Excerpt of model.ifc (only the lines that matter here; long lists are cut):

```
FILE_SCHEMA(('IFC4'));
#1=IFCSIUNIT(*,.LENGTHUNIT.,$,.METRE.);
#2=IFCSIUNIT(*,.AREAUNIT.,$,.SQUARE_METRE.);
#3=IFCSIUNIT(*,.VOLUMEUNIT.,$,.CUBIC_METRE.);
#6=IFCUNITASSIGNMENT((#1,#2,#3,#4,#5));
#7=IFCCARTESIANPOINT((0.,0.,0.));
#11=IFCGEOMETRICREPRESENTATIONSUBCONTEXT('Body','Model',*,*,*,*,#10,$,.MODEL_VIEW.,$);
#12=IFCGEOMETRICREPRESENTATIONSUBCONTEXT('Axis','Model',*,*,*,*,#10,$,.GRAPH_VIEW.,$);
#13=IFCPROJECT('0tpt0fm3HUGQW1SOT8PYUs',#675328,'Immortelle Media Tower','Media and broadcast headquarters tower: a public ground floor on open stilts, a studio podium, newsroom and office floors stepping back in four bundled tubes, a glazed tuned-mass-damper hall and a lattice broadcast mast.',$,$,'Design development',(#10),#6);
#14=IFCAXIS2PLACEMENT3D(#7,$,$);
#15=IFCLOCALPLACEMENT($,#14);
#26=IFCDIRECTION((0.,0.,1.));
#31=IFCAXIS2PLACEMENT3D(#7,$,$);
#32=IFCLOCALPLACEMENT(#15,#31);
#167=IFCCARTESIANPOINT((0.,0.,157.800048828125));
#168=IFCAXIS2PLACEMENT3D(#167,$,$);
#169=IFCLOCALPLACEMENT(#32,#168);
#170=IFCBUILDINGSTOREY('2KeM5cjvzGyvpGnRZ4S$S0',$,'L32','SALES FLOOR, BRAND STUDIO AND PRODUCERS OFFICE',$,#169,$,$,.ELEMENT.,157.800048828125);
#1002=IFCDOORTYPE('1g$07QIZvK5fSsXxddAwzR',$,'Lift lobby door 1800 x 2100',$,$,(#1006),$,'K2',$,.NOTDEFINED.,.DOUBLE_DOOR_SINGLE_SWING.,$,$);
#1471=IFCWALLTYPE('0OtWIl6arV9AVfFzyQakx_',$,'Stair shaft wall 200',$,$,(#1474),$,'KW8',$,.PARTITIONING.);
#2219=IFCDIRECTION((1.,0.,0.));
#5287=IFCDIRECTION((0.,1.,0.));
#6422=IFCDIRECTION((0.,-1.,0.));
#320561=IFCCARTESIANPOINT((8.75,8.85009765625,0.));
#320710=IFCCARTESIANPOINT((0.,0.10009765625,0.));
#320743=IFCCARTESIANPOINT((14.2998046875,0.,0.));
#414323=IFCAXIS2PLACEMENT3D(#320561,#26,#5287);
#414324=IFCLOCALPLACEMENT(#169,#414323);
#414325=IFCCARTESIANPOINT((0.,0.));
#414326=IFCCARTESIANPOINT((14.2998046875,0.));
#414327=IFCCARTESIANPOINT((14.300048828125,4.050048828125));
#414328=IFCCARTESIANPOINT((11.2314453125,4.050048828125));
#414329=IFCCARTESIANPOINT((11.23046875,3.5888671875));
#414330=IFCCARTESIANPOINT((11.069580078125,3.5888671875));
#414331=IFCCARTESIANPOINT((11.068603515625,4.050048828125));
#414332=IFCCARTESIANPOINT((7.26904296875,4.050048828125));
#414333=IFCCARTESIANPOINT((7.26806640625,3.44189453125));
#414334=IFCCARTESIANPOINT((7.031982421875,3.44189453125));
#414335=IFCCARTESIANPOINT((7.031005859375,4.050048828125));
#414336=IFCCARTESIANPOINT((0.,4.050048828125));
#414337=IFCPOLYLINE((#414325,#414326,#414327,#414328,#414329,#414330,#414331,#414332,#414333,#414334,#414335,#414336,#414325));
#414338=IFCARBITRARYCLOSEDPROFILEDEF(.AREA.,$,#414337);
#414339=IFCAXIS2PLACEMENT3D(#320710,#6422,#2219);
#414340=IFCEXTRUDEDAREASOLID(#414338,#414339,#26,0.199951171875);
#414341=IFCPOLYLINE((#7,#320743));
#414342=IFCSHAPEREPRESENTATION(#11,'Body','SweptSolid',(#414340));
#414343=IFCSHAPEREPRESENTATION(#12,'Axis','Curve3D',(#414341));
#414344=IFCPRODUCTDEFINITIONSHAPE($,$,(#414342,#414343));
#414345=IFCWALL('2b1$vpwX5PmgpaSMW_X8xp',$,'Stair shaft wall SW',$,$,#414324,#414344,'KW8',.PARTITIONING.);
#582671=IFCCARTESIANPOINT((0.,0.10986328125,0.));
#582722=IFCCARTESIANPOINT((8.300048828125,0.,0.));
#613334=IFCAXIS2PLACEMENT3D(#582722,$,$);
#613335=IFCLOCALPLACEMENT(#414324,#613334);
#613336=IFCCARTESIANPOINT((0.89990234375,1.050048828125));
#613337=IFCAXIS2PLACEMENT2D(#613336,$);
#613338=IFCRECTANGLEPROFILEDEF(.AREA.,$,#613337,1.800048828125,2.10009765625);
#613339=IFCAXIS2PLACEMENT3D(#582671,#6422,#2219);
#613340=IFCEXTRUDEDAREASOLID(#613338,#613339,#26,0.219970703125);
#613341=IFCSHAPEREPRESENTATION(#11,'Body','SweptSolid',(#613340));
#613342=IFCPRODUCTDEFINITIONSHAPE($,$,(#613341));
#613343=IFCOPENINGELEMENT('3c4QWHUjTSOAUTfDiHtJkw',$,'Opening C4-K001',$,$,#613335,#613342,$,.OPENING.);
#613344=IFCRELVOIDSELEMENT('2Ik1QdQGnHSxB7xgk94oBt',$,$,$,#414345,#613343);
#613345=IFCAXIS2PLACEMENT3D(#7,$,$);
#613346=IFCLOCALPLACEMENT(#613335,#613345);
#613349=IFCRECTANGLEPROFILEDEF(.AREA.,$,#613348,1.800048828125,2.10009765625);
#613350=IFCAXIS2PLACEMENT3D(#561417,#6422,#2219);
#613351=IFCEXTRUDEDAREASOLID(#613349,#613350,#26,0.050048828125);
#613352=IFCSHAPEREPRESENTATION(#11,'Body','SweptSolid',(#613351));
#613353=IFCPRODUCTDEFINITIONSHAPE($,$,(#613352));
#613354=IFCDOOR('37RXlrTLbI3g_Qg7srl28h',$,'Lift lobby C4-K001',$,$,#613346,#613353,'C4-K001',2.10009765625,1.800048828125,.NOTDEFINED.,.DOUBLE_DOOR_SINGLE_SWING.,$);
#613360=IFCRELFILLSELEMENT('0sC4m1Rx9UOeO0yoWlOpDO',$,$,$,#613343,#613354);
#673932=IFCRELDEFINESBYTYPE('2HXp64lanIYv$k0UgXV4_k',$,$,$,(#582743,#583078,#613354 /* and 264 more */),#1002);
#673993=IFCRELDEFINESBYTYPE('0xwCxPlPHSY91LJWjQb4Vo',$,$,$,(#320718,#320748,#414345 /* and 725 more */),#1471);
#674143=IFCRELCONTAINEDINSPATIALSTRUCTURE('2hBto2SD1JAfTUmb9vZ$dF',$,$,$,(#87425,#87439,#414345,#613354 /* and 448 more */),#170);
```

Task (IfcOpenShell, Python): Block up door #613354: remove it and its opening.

```python
import ifcopenshell
import ifcopenshell.api.feature
import ifcopenshell.api.root
import ifcopenshell.geom
import ifcopenshell.util.shape

model = ifcopenshell.open("model.ifc")
settings = ifcopenshell.geom.settings()


def volume(element):
    """Net volume in cubic metres, openings subtracted."""
    shape = ifcopenshell.geom.create_shape(settings, element)
    return ifcopenshell.util.shape.get_volume(shape.geometry)


door = model.by_guid("37RXlrTLbI3g_Qg7srl28h")
opening = door.FillsVoids[0].RelatingOpeningElement
wall = opening.VoidsElements[0].RelatingBuildingElement
before = volume(wall)

ifcopenshell.api.root.remove_product(model, product=door)
ifcopenshell.api.feature.remove_feature(model, feature=opening)

after = volume(wall)

print(f"wall volume {before:.3f} -> {after:.3f} m3")

model.write("model_v2.ifc")
```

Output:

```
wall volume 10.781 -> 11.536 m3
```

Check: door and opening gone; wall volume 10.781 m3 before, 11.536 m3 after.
